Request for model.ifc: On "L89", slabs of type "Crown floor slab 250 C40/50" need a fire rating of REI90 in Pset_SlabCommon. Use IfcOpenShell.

First a look at what the model holds.

```python
import ifcopenshell
import ifcopenshell.util.element

model = ifcopenshell.open("model.ifc")
print(model.schema)
storey = next(s for s in model.by_type("IfcBuildingStorey") if s.Name == "L89")
slabs = [e for e in ifcopenshell.util.element.get_decomposition(storey) if e.is_a("IfcSlab")]
seen = {}
for e in slabs:
    element_type = ifcopenshell.util.element.get_type(e)
    key = (element_type.Name if element_type != e and element_type else None, ifcopenshell.util.element.get_pset(e, "Pset_SlabCommon", "FireRating"))
    seen[key] = seen.get(key, 0) + 1
for (name, value), count in sorted(seen.items(), key=str):
    print(count, "x", name, "|", value)
```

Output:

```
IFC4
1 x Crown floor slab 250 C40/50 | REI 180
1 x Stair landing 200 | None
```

```python
import ifcopenshell
import ifcopenshell.api.pset
import ifcopenshell.util.element

model = ifcopenshell.open("model.ifc")

storey = next(s for s in model.by_type("IfcBuildingStorey") if s.Name == "L89")
slabs = [e for e in ifcopenshell.util.element.get_decomposition(storey) if e.is_a("IfcSlab")]

count = 0
for e in slabs:
    element_type = ifcopenshell.util.element.get_type(e)
    if element_type in (None, e) or element_type.Name != "Crown floor slab 250 C40/50":
        continue
    found = ifcopenshell.util.element.get_pset(e, "Pset_SlabCommon", should_inherit=False)
    if found:
        pset = model.by_id(found["id"])
        if len(ifcopenshell.util.element.get_elements_by_pset(pset)) > 1:
            pset = ifcopenshell.api.pset.unshare_pset(model, products=[e], pset=pset)[0]
    else:
        pset = ifcopenshell.api.pset.add_pset(model, product=e, name="Pset_SlabCommon")
    ifcopenshell.api.pset.edit_pset(model, pset=pset, properties={"FireRating": "REI90"})
    count += 1

print(count, "slabs updated")

model.write("model_rev.ifc")
```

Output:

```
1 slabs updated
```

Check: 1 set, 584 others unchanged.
